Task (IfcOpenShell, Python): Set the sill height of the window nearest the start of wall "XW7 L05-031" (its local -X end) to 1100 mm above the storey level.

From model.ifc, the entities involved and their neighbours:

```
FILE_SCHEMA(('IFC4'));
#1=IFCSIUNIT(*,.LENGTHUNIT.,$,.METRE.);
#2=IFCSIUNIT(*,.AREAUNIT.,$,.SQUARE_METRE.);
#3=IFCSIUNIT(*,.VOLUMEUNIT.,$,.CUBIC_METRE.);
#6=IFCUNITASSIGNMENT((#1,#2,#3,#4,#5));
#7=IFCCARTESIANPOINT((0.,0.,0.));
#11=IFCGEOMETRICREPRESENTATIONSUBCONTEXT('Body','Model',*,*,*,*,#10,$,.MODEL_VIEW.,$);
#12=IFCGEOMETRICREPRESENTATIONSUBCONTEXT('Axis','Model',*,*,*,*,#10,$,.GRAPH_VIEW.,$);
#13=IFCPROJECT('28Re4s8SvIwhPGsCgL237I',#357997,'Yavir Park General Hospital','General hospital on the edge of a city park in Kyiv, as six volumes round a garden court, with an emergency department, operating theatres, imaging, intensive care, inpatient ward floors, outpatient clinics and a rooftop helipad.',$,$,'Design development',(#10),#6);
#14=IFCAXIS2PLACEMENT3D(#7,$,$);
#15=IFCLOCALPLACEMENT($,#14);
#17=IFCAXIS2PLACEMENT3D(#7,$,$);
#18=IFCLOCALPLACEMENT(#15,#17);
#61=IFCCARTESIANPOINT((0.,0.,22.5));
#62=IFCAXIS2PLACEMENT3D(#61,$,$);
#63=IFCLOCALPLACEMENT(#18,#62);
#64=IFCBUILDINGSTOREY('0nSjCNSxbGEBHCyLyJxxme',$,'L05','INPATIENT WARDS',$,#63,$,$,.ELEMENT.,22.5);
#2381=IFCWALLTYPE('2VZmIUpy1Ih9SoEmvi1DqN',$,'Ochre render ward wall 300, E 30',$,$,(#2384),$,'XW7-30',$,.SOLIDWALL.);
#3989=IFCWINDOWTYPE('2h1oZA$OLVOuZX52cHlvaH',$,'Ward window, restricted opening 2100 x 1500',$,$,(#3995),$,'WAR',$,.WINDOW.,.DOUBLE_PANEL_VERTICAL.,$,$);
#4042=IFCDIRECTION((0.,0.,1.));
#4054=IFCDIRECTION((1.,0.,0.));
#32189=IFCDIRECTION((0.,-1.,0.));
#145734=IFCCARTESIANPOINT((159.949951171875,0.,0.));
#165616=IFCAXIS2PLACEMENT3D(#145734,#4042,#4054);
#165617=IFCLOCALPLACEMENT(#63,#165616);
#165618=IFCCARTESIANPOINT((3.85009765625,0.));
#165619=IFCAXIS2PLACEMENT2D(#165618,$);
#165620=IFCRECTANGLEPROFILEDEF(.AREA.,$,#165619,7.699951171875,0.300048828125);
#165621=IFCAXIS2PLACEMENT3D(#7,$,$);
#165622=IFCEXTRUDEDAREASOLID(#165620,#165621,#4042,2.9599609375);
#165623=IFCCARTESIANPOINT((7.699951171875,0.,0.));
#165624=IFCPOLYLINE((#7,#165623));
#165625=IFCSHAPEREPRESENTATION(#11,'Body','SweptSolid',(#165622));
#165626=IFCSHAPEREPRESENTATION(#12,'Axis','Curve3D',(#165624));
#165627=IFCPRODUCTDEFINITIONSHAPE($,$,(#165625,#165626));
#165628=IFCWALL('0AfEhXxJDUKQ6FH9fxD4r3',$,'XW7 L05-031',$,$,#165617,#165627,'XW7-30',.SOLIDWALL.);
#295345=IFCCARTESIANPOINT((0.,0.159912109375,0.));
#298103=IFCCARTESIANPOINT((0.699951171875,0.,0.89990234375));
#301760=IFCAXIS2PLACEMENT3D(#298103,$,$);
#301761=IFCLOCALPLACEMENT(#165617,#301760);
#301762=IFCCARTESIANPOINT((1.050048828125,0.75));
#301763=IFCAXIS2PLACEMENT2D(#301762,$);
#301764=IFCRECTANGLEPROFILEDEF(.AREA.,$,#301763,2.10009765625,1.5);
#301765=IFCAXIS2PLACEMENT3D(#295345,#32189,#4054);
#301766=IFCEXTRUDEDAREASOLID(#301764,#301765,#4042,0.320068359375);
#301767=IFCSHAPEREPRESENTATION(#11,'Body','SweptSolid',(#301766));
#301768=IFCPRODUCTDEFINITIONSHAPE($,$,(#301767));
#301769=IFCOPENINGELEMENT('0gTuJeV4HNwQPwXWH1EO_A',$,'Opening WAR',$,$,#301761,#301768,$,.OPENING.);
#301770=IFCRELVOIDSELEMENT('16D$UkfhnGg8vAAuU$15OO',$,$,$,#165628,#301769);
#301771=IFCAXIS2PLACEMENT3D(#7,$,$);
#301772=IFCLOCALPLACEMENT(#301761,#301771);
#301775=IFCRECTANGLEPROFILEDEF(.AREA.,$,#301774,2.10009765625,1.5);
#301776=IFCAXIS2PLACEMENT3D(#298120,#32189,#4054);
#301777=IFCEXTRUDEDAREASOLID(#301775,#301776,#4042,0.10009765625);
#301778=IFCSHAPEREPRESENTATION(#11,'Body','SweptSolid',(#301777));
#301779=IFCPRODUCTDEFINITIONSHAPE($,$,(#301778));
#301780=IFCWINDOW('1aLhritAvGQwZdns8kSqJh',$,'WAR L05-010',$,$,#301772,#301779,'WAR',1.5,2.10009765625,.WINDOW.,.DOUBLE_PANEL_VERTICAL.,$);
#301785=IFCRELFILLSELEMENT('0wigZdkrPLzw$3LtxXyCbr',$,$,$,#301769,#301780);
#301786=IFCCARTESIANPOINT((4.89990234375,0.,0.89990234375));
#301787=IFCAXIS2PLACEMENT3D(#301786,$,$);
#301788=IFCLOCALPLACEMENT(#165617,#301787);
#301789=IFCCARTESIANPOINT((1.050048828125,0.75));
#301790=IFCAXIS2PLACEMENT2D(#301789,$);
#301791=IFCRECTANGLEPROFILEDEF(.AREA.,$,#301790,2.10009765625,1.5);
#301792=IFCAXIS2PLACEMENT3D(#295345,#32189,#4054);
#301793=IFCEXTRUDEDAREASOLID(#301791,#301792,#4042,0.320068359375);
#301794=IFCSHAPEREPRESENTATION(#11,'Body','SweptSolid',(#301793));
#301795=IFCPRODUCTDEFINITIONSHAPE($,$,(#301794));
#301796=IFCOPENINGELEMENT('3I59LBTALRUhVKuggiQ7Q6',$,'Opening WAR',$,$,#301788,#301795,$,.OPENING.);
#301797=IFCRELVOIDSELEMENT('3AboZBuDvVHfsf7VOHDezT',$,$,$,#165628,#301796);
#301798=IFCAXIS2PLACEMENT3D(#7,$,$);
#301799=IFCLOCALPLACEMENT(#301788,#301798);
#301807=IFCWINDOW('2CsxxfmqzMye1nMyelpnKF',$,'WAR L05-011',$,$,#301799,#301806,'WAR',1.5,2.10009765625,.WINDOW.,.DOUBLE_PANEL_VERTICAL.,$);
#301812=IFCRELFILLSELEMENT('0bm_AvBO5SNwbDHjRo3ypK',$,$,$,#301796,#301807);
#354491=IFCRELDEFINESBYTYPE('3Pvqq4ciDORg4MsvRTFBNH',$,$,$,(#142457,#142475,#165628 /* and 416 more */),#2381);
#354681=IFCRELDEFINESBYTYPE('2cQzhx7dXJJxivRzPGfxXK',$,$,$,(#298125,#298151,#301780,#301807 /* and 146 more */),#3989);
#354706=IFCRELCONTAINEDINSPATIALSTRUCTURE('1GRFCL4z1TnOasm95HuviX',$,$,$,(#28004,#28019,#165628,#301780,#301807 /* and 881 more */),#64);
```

```python
import numpy as np
import ifcopenshell
import ifcopenshell.api.geometry
import ifcopenshell.geom
import ifcopenshell.util.element
import ifcopenshell.util.placement
import ifcopenshell.util.shape
import ifcopenshell.util.unit

model = ifcopenshell.open("model.ifc")
unit_scale = ifcopenshell.util.unit.calculate_unit_scale(model)

window = model.by_id(301780)
opening = window.FillsVoids[0].RelatingOpeningElement
storey = ifcopenshell.util.element.get_container(window, ifc_class="IfcBuildingStorey")
level = ifcopenshell.util.placement.get_local_placement(storey.ObjectPlacement)[2, 3]

# The opening's origin need not be at the sill, so measure its lowest point.
shape = ifcopenshell.geom.create_shape(ifcopenshell.geom.settings(), opening)
bottom = ifcopenshell.util.shape.get_shape_bottom_elevation(shape, shape.geometry) / unit_scale
dz = level + 1.1 - bottom

shift = np.array([0.0, 0.0, dz])
# The window is placed relative to its opening, so it follows when the opening moves.
matrix = ifcopenshell.util.placement.get_local_placement(opening.ObjectPlacement)
matrix[:3, 3] += shift
ifcopenshell.api.geometry.edit_object_placement(
    model, product=opening, matrix=matrix, is_si=False, should_transform_children=True
)

print(f"moved by {dz * unit_scale:+.3f} m")

model.write("model_updated.ifc")
```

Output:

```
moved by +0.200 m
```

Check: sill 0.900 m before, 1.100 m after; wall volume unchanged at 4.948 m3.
